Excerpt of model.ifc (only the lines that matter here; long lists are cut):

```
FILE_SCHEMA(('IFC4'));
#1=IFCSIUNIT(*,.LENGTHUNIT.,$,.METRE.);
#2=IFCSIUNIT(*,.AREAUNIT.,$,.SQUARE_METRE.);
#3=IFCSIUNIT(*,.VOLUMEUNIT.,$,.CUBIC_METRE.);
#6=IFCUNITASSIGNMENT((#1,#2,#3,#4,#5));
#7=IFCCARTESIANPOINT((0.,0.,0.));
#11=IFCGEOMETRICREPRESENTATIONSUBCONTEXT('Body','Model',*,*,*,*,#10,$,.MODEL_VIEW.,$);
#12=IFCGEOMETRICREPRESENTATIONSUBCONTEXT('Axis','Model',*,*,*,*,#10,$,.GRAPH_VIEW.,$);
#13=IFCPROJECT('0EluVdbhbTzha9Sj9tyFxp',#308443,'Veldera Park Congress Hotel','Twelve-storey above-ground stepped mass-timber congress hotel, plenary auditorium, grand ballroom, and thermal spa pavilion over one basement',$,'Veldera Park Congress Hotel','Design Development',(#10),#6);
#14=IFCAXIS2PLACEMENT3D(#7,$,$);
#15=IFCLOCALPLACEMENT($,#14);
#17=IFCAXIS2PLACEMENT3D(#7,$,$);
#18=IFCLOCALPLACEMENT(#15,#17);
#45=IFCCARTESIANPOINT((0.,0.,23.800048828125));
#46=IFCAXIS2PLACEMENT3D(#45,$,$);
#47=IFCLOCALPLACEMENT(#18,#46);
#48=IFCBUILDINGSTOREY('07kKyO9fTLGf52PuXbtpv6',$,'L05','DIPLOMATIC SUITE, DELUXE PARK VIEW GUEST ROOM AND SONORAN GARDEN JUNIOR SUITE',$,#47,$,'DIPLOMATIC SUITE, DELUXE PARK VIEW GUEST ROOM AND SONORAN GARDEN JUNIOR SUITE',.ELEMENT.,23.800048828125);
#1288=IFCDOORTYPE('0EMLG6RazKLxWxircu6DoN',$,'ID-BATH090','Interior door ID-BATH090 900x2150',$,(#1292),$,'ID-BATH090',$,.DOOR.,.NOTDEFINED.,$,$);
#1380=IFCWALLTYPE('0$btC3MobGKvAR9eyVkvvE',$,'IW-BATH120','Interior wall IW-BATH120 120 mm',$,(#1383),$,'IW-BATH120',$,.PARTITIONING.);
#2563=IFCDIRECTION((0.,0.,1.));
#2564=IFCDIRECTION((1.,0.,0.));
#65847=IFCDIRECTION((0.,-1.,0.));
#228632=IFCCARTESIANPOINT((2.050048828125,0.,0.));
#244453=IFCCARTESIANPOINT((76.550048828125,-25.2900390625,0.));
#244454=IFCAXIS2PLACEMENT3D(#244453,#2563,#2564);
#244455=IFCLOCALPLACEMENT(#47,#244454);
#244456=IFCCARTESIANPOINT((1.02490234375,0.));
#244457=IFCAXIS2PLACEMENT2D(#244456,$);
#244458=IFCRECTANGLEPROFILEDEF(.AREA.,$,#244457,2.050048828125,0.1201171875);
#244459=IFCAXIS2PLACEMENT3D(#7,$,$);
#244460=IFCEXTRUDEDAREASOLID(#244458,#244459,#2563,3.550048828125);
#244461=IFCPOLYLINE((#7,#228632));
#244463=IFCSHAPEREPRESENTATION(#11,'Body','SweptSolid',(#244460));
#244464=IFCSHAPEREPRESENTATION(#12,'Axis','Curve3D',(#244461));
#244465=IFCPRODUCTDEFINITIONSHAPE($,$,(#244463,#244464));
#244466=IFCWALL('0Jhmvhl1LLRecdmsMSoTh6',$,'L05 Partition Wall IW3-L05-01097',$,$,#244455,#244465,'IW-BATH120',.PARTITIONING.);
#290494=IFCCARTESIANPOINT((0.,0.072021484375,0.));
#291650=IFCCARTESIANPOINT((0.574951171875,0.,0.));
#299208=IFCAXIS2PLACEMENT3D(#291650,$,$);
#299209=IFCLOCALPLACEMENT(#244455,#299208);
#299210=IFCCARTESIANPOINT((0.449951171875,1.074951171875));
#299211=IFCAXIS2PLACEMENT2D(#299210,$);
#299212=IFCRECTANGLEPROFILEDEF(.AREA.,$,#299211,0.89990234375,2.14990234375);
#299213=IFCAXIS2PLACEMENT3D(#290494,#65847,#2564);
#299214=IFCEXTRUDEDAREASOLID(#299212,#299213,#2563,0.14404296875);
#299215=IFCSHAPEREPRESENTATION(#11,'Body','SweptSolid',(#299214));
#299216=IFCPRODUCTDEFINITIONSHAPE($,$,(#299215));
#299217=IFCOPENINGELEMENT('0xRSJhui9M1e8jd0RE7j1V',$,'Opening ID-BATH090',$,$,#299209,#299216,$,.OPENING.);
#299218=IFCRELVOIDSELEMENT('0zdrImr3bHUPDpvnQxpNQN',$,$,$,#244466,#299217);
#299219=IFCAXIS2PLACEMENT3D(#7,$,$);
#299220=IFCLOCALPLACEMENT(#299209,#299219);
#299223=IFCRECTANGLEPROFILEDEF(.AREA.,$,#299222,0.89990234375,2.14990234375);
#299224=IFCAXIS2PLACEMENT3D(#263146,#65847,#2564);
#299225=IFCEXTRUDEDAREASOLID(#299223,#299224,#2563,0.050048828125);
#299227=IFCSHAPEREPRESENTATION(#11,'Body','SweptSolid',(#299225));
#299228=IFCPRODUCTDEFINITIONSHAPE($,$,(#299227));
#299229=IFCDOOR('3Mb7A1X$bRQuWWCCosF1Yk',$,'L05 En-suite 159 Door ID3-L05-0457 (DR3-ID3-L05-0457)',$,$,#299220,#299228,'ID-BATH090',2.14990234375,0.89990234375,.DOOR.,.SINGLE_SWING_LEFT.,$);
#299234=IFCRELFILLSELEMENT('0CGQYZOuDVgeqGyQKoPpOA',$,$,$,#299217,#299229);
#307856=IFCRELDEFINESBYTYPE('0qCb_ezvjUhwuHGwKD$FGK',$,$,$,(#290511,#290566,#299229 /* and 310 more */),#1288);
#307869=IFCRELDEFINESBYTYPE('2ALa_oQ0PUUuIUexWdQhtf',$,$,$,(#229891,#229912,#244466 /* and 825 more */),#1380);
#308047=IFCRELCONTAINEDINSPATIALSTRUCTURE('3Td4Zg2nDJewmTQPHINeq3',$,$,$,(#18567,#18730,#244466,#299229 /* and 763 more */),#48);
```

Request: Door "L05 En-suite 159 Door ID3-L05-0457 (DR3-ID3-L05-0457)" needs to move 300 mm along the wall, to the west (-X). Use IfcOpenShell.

```python
import ifcopenshell
import ifcopenshell.api.geometry
import ifcopenshell.util.placement

model = ifcopenshell.open("model.ifc")

door = model.by_guid("3Mb7A1X$bRQuWWCCosF1Yk")
opening = door.FillsVoids[0].RelatingOpeningElement
wall = opening.VoidsElements[0].RelatingBuildingElement

wall_matrix = ifcopenshell.util.placement.get_local_placement(wall.ObjectPlacement)
shift = wall_matrix[:3, 0] * -0.3
before = ifcopenshell.util.placement.get_local_placement(door.ObjectPlacement)[:3, 3].copy()

# The door is placed relative to its opening, so it follows when the opening moves.
matrix = ifcopenshell.util.placement.get_local_placement(opening.ObjectPlacement)
matrix[:3, 3] += shift
ifcopenshell.api.geometry.edit_object_placement(
    model, product=opening, matrix=matrix, is_si=False, should_transform_children=True
)

after = ifcopenshell.util.placement.get_local_placement(door.ObjectPlacement)[:3, 3]
print("door moved by", (after - before).round(3) + 0.0)

model.write("model_updated.ifc")
```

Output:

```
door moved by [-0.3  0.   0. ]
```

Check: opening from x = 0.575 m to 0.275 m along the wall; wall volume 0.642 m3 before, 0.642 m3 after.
